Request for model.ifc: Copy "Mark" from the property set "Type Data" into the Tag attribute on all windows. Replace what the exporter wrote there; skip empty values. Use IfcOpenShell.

First a look at what the model holds.

```python
import ifcopenshell
import ifcopenshell.util.element

model = ifcopenshell.open("model.ifc")
print(model.schema)
windows = model.by_type("IfcWindow")
print(len(windows), "windows")
for e in windows[:8]:
    source = ifcopenshell.util.element.get_pset(e, "Type Data", "Mark")
    target = e.Tag
    print(e.id(), repr(source), repr(target), sep=" | ")
```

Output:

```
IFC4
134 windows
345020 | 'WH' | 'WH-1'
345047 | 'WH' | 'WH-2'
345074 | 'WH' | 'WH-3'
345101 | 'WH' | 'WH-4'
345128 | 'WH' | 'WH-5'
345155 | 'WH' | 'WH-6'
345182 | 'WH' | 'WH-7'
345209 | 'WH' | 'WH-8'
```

```python
import ifcopenshell
import ifcopenshell.util.element

model = ifcopenshell.open("model.ifc")

count = 0
for e in model.by_type("IfcWindow"):
    value = ifcopenshell.util.element.get_pset(e, "Type Data", "Mark")
    current = e.Tag
    if not value or not value.strip() or current == value:
        continue
    e.Tag = value
    count += 1

print(count, "windows updated")

model.write("model_edited.ifc")
```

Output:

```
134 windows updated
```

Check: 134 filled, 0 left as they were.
